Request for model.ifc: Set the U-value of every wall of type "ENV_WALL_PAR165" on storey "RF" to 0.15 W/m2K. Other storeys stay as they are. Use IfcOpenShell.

First a look at what the model holds.

```python
import ifcopenshell
import ifcopenshell.util.element

model = ifcopenshell.open("model.ifc")
print(model.schema)
storey = next(s for s in model.by_type("IfcBuildingStorey") if s.Name == "RF")
walls = [e for e in ifcopenshell.util.element.get_decomposition(storey) if e.is_a("IfcWall")]
seen = {}
for e in walls:
    element_type = ifcopenshell.util.element.get_type(e)
    key = (element_type.Name if element_type != e and element_type else None, ifcopenshell.util.element.get_pset(e, "Pset_WallCommon", "ThermalTransmittance"))
    seen[key] = seen.get(key, 0) + 1
for (name, value), count in sorted(seen.items(), key=str):
    print(count, "x", name, "|", value)
```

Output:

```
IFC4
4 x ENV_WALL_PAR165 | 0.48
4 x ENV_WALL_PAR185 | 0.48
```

```python
import ifcopenshell
import ifcopenshell.api.pset
import ifcopenshell.util.element

model = ifcopenshell.open("model.ifc")

storey = next(s for s in model.by_type("IfcBuildingStorey") if s.Name == "RF")
walls = [e for e in ifcopenshell.util.element.get_decomposition(storey) if e.is_a("IfcWall")]

count = 0
for e in walls:
    element_type = ifcopenshell.util.element.get_type(e)
    if element_type in (None, e) or element_type.Name != "ENV_WALL_PAR165":
        continue
    # add_pset returns the element's existing set when there is one.
    pset = ifcopenshell.api.pset.add_pset(model, product=e, name="Pset_WallCommon")
    ifcopenshell.api.pset.edit_pset(model, pset=pset, properties={"ThermalTransmittance": 0.15})
    count += 1

print(count, "walls updated")

model.write("model_edited.ifc")
```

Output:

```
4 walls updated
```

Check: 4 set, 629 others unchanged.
